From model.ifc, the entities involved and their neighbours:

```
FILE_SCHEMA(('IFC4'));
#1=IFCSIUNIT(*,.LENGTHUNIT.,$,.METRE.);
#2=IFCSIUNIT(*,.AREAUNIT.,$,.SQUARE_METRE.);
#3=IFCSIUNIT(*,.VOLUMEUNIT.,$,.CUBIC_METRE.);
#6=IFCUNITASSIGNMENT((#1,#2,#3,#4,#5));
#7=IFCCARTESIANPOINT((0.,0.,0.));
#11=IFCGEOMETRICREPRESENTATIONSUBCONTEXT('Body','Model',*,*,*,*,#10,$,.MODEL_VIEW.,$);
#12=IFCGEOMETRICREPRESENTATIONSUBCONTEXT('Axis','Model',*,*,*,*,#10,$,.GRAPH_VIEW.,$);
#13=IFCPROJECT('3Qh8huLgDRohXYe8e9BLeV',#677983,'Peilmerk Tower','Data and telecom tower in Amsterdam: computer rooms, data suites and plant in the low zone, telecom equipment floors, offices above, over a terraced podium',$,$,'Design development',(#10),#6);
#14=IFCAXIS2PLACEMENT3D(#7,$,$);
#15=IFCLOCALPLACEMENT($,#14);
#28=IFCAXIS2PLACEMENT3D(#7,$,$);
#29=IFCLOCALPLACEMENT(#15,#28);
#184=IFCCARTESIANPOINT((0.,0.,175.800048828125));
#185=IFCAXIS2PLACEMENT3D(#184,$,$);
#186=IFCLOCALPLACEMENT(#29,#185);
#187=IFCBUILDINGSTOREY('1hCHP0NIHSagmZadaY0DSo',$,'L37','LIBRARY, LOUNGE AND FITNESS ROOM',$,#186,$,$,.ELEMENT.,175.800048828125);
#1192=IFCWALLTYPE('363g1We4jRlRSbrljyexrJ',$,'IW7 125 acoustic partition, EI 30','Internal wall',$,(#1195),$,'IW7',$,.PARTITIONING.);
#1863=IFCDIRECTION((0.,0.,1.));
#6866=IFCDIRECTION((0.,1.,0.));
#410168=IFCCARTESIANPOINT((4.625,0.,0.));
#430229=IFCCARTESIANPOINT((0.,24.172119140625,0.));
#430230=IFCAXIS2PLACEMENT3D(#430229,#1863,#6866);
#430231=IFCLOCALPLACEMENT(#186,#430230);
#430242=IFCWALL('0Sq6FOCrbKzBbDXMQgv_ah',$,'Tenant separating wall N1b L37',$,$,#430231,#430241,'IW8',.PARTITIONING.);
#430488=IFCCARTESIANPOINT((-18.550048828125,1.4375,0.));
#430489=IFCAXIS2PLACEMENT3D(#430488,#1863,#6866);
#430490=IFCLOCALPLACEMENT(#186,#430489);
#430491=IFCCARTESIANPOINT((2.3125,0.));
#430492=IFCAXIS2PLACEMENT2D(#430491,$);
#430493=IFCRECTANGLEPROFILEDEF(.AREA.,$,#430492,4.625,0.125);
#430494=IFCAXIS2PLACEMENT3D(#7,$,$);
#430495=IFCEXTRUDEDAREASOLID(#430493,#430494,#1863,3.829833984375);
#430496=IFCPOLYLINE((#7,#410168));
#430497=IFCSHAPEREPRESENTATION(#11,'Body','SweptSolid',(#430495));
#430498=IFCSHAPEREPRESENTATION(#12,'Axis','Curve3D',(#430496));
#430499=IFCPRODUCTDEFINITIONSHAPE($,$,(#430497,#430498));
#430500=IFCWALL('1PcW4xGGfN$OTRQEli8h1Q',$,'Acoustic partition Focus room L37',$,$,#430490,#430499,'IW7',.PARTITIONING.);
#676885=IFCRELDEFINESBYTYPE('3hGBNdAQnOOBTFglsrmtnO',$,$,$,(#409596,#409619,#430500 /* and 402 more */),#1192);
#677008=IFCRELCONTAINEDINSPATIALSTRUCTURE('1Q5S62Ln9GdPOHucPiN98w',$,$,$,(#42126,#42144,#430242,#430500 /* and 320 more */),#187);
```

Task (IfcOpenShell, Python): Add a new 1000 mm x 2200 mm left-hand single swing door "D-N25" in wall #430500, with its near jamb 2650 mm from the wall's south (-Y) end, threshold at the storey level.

```python
import numpy as np
import ifcopenshell
import ifcopenshell.api.feature
import ifcopenshell.api.geometry
import ifcopenshell.api.root
import ifcopenshell.api.spatial
import ifcopenshell.geom
import ifcopenshell.util.element
import ifcopenshell.util.placement
import ifcopenshell.util.representation
import ifcopenshell.util.shape
import ifcopenshell.util.unit

model = ifcopenshell.open("model.ifc")
unit_scale = ifcopenshell.util.unit.calculate_unit_scale(model)
settings = ifcopenshell.geom.settings()


def volume(element):
    """Net volume in cubic metres, openings subtracted."""
    shape = ifcopenshell.geom.create_shape(settings, element)
    return ifcopenshell.util.shape.get_volume(shape.geometry)


wall = model.by_id(430500)
storey = ifcopenshell.util.element.get_container(wall, ifc_class="IfcBuildingStorey")
context = ifcopenshell.util.representation.get_context(model, "Model", "Body", "MODEL_VIEW")
before = volume(wall)

width, height, from_end, sill = 1, 2.2, 2.65, 0.0  # metres

# The wall runs along its own X axis, and the end named is its -X end.
wall_shape = ifcopenshell.geom.create_shape(settings, wall)
x, y, z = ifcopenshell.util.shape.get_vertices(wall_shape.geometry).T
start = x.min() + from_end
face, thickness = float(y.min()), float(y.max() - y.min())
wall_matrix = ifcopenshell.util.placement.get_local_placement(wall.ObjectPlacement)
level = ifcopenshell.util.placement.get_local_placement(storey.ObjectPlacement)[2, 3]


def in_wall(x, y):
    """Placement at x, y metres in the wall's axes, at sill height."""
    matrix = wall_matrix.copy()
    matrix[:, 3] = wall_matrix @ np.array([x / unit_scale, y / unit_scale, 0.0, 1.0])
    matrix[2, 3] = level + sill / unit_scale
    return matrix


# Opening: a box that overshoots both wall faces by 50 mm.
opening = ifcopenshell.api.root.create_entity(model, ifc_class="IfcOpeningElement", predefined_type="OPENING")
box = ifcopenshell.api.geometry.add_wall_representation(
    model, context=context, length=width, height=height, thickness=thickness + 0.1
)
ifcopenshell.api.geometry.assign_representation(model, product=opening, representation=box)
ifcopenshell.api.geometry.edit_object_placement(model, product=opening, matrix=in_wall(start, face - 0.05), is_si=False)
ifcopenshell.api.feature.add_feature(model, feature=opening, element=wall)

door = ifcopenshell.api.root.create_entity(model, ifc_class="IfcDoor", name="D-N25", predefined_type="DOOR")
door.OverallWidth, door.OverallHeight = width / unit_scale, height / unit_scale
door.OperationType = "SINGLE_SWING_LEFT"
body = ifcopenshell.api.geometry.add_door_representation(
    model,
    context=context,
    overall_width=door.OverallWidth,
    overall_height=door.OverallHeight,
    operation_type="SINGLE_SWING_LEFT",
    lining_properties={"LiningDepth": thickness / unit_scale, "ThresholdDepth": thickness / unit_scale},
)
ifcopenshell.api.geometry.assign_representation(model, product=door, representation=body)
ifcopenshell.api.spatial.assign_container(model, products=[door], relating_structure=storey)
ifcopenshell.api.feature.add_filling(model, opening=opening, element=door)

# The lining spans the wall, so the door starts at the wall face.
ifcopenshell.api.geometry.edit_object_placement(model, product=door, matrix=in_wall(start, face), is_si=False)

after = volume(wall)

print(f"wall volume {before:.3f} -> {after:.3f} m3")

model.write("model_rev.ifc")
```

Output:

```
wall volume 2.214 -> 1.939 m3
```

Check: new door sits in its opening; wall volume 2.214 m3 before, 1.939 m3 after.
